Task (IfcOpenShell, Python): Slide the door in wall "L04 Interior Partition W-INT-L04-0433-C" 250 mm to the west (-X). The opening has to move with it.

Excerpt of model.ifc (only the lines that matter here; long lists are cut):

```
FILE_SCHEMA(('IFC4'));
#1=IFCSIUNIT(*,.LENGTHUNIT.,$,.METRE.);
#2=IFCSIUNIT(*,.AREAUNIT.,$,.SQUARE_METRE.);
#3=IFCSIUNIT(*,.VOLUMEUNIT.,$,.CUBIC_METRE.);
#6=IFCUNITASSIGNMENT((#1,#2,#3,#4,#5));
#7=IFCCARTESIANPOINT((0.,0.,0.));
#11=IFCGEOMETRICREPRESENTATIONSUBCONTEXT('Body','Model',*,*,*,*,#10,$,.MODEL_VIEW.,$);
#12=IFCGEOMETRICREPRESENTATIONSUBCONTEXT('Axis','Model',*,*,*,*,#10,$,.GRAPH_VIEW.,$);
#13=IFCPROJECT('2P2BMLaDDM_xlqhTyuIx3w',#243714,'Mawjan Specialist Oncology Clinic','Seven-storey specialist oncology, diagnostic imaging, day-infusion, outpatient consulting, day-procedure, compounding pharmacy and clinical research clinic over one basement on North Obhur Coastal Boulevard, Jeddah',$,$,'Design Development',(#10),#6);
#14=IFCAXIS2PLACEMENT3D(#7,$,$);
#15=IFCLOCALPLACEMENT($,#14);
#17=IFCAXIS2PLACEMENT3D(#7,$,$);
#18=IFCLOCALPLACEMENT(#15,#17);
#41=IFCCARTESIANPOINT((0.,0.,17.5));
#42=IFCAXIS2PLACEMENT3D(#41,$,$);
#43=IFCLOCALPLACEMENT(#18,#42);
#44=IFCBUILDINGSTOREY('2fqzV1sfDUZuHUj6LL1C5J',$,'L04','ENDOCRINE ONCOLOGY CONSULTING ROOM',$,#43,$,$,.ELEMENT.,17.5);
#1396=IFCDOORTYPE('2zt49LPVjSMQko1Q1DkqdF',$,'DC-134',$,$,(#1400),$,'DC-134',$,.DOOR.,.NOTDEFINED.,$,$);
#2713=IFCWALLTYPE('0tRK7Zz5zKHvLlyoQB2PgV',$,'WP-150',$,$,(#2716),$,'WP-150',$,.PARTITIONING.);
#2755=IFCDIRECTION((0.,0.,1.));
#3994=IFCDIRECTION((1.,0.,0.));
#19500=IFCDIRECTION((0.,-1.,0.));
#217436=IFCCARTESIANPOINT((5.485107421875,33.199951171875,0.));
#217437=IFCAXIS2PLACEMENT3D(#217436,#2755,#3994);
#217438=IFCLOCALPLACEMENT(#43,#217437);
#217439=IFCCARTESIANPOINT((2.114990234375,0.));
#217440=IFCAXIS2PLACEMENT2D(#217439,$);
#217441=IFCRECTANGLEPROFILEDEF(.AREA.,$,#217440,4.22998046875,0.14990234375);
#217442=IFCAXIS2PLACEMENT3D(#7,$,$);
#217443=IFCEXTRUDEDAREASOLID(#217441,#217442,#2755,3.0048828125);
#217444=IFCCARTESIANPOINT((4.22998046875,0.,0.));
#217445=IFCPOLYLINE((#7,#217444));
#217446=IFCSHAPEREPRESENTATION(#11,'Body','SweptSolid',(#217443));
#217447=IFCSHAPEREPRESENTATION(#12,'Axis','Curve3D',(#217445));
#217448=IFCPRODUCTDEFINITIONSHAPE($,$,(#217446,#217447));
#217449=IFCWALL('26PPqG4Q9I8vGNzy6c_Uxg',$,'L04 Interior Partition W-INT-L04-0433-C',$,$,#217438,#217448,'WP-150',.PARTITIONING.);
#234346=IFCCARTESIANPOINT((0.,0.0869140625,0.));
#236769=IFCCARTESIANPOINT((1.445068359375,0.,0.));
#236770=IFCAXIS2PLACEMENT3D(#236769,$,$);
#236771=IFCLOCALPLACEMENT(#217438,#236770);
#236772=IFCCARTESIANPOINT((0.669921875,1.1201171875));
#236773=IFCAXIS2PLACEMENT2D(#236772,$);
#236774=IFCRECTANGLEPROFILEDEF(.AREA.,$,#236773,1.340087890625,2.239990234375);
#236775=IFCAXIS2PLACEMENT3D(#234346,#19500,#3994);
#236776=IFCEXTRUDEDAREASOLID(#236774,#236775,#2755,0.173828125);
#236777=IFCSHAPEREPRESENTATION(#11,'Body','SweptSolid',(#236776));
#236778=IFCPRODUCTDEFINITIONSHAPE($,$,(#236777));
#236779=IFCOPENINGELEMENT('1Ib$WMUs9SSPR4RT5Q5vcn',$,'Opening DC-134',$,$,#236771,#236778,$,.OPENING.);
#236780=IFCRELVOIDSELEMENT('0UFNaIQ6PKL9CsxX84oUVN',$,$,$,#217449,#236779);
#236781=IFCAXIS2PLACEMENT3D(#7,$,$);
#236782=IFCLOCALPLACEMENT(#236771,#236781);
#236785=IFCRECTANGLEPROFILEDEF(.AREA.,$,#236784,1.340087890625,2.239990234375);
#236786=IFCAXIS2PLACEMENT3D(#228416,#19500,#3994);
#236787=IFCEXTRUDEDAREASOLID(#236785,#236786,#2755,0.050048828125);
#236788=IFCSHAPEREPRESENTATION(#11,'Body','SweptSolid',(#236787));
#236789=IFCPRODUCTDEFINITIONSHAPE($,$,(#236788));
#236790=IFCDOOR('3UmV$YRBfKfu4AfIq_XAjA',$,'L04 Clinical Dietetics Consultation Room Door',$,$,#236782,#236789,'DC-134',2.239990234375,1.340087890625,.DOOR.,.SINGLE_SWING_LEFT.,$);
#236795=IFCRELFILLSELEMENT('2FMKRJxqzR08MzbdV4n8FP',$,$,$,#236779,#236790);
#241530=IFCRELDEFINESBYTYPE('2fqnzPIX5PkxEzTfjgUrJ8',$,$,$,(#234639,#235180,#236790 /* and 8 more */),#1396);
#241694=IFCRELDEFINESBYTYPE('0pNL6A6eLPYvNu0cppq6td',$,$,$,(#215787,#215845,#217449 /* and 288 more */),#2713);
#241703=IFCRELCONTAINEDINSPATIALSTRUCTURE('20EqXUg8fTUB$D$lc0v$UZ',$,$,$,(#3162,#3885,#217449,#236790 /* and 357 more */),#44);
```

```python
import ifcopenshell
import ifcopenshell.api.geometry
import ifcopenshell.util.placement
import ifcopenshell.util.unit

model = ifcopenshell.open("model.ifc")
unit_scale = ifcopenshell.util.unit.calculate_unit_scale(model)

door = model.by_id(236790)
opening = door.FillsVoids[0].RelatingOpeningElement
wall = opening.VoidsElements[0].RelatingBuildingElement

wall_matrix = ifcopenshell.util.placement.get_local_placement(wall.ObjectPlacement)
shift = wall_matrix[:3, 0] * -0.25 / unit_scale
before = ifcopenshell.util.placement.get_local_placement(door.ObjectPlacement)[:3, 3].copy()

# The door is placed relative to its opening, so it follows when the opening moves.
matrix = ifcopenshell.util.placement.get_local_placement(opening.ObjectPlacement)
matrix[:3, 3] += shift
ifcopenshell.api.geometry.edit_object_placement(
    model, product=opening, matrix=matrix, is_si=False, should_transform_children=True
)

after = ifcopenshell.util.placement.get_local_placement(door.ObjectPlacement)[:3, 3]
print("door moved by", (after - before).round(3) + 0.0)

model.write("model_rev.ifc")
```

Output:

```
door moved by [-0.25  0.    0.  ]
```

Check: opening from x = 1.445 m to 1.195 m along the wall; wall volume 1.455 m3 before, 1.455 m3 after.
